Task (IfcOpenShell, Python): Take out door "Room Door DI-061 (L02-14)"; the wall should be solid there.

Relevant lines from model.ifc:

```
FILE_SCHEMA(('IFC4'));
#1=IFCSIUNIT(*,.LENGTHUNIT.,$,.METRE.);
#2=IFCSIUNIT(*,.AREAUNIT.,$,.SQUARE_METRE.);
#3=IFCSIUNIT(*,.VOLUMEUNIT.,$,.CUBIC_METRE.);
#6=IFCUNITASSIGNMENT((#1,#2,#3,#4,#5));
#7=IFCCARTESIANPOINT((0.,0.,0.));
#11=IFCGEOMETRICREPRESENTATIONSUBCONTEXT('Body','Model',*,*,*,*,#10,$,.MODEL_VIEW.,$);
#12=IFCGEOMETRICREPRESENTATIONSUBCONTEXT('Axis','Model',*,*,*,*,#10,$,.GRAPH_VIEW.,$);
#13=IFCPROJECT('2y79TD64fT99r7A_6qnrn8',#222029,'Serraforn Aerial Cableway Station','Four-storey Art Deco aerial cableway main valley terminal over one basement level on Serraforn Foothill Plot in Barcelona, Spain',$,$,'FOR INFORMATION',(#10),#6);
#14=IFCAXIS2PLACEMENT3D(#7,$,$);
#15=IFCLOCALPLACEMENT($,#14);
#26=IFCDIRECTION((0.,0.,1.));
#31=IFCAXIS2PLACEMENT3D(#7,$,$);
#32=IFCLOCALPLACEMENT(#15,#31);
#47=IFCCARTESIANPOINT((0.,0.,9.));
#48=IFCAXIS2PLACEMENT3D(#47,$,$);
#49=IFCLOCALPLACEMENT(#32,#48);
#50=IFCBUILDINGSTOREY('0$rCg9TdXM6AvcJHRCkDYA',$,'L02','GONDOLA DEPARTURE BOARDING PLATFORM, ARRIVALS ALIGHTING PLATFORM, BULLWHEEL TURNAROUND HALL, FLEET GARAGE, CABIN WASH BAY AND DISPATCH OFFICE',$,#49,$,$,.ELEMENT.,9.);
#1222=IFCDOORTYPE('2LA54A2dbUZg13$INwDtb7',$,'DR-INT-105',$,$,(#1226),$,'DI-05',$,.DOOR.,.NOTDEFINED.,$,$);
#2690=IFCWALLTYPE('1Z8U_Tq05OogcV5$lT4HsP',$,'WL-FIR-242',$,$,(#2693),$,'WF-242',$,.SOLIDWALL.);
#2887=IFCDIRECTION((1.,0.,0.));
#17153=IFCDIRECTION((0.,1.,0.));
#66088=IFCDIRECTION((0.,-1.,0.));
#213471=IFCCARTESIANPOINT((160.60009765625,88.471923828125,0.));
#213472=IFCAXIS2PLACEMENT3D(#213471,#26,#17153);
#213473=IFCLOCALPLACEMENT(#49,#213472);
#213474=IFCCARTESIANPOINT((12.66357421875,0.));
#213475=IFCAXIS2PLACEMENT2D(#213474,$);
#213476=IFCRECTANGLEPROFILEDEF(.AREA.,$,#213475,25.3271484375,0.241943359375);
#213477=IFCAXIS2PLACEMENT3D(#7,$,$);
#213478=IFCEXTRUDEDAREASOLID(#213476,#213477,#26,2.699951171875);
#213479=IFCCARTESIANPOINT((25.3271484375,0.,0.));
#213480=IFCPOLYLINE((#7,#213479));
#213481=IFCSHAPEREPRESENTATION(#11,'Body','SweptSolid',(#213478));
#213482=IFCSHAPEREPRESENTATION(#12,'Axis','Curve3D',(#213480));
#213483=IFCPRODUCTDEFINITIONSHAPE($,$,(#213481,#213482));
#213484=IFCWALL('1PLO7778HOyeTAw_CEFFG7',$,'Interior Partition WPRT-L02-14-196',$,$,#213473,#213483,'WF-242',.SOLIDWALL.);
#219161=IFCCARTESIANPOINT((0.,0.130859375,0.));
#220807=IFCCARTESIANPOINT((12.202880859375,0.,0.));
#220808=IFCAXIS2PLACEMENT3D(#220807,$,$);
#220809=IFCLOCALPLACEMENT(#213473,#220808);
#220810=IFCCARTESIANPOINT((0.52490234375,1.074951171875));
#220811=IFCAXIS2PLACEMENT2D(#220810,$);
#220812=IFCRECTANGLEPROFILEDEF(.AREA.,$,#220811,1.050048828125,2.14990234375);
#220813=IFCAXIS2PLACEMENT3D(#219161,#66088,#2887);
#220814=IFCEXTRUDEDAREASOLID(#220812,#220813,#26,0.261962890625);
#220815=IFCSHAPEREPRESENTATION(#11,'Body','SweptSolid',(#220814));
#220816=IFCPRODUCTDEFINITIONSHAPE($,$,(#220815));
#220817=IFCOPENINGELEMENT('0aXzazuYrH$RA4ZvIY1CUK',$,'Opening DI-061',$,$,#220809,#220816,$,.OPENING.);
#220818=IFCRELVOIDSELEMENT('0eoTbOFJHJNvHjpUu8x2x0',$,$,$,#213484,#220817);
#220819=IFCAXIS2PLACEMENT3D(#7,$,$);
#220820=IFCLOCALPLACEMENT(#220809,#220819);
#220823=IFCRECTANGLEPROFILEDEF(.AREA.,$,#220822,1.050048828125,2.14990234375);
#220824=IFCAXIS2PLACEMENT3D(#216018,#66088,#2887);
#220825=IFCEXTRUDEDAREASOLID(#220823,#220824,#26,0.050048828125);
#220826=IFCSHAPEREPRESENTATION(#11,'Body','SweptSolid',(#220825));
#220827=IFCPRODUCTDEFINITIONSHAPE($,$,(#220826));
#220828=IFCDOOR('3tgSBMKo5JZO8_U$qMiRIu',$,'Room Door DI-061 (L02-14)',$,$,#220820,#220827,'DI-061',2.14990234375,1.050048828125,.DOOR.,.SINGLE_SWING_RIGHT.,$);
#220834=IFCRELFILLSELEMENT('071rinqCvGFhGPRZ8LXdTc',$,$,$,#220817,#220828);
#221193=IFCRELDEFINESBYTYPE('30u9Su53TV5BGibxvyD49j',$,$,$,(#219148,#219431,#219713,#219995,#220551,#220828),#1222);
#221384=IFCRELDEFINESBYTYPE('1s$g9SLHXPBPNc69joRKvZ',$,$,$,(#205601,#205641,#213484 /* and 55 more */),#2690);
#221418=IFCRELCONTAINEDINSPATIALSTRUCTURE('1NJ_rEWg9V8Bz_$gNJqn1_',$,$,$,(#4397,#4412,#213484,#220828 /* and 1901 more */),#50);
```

```python
import ifcopenshell
import ifcopenshell.api.feature
import ifcopenshell.api.root
import ifcopenshell.geom
import ifcopenshell.util.shape

model = ifcopenshell.open("model.ifc")
settings = ifcopenshell.geom.settings()


def volume(element):
    """Net volume in cubic metres, openings subtracted."""
    shape = ifcopenshell.geom.create_shape(settings, element)
    return ifcopenshell.util.shape.get_volume(shape.geometry)


door = model.by_guid("3tgSBMKo5JZO8_U$qMiRIu")
opening = door.FillsVoids[0].RelatingOpeningElement
wall = opening.VoidsElements[0].RelatingBuildingElement
before = volume(wall)

ifcopenshell.api.root.remove_product(model, product=door)
ifcopenshell.api.feature.remove_feature(model, feature=opening)

after = volume(wall)

print(f"wall volume {before:.3f} -> {after:.3f} m3")

model.write("model_rev.ifc")
```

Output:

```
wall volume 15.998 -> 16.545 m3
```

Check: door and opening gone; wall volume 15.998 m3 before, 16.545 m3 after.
